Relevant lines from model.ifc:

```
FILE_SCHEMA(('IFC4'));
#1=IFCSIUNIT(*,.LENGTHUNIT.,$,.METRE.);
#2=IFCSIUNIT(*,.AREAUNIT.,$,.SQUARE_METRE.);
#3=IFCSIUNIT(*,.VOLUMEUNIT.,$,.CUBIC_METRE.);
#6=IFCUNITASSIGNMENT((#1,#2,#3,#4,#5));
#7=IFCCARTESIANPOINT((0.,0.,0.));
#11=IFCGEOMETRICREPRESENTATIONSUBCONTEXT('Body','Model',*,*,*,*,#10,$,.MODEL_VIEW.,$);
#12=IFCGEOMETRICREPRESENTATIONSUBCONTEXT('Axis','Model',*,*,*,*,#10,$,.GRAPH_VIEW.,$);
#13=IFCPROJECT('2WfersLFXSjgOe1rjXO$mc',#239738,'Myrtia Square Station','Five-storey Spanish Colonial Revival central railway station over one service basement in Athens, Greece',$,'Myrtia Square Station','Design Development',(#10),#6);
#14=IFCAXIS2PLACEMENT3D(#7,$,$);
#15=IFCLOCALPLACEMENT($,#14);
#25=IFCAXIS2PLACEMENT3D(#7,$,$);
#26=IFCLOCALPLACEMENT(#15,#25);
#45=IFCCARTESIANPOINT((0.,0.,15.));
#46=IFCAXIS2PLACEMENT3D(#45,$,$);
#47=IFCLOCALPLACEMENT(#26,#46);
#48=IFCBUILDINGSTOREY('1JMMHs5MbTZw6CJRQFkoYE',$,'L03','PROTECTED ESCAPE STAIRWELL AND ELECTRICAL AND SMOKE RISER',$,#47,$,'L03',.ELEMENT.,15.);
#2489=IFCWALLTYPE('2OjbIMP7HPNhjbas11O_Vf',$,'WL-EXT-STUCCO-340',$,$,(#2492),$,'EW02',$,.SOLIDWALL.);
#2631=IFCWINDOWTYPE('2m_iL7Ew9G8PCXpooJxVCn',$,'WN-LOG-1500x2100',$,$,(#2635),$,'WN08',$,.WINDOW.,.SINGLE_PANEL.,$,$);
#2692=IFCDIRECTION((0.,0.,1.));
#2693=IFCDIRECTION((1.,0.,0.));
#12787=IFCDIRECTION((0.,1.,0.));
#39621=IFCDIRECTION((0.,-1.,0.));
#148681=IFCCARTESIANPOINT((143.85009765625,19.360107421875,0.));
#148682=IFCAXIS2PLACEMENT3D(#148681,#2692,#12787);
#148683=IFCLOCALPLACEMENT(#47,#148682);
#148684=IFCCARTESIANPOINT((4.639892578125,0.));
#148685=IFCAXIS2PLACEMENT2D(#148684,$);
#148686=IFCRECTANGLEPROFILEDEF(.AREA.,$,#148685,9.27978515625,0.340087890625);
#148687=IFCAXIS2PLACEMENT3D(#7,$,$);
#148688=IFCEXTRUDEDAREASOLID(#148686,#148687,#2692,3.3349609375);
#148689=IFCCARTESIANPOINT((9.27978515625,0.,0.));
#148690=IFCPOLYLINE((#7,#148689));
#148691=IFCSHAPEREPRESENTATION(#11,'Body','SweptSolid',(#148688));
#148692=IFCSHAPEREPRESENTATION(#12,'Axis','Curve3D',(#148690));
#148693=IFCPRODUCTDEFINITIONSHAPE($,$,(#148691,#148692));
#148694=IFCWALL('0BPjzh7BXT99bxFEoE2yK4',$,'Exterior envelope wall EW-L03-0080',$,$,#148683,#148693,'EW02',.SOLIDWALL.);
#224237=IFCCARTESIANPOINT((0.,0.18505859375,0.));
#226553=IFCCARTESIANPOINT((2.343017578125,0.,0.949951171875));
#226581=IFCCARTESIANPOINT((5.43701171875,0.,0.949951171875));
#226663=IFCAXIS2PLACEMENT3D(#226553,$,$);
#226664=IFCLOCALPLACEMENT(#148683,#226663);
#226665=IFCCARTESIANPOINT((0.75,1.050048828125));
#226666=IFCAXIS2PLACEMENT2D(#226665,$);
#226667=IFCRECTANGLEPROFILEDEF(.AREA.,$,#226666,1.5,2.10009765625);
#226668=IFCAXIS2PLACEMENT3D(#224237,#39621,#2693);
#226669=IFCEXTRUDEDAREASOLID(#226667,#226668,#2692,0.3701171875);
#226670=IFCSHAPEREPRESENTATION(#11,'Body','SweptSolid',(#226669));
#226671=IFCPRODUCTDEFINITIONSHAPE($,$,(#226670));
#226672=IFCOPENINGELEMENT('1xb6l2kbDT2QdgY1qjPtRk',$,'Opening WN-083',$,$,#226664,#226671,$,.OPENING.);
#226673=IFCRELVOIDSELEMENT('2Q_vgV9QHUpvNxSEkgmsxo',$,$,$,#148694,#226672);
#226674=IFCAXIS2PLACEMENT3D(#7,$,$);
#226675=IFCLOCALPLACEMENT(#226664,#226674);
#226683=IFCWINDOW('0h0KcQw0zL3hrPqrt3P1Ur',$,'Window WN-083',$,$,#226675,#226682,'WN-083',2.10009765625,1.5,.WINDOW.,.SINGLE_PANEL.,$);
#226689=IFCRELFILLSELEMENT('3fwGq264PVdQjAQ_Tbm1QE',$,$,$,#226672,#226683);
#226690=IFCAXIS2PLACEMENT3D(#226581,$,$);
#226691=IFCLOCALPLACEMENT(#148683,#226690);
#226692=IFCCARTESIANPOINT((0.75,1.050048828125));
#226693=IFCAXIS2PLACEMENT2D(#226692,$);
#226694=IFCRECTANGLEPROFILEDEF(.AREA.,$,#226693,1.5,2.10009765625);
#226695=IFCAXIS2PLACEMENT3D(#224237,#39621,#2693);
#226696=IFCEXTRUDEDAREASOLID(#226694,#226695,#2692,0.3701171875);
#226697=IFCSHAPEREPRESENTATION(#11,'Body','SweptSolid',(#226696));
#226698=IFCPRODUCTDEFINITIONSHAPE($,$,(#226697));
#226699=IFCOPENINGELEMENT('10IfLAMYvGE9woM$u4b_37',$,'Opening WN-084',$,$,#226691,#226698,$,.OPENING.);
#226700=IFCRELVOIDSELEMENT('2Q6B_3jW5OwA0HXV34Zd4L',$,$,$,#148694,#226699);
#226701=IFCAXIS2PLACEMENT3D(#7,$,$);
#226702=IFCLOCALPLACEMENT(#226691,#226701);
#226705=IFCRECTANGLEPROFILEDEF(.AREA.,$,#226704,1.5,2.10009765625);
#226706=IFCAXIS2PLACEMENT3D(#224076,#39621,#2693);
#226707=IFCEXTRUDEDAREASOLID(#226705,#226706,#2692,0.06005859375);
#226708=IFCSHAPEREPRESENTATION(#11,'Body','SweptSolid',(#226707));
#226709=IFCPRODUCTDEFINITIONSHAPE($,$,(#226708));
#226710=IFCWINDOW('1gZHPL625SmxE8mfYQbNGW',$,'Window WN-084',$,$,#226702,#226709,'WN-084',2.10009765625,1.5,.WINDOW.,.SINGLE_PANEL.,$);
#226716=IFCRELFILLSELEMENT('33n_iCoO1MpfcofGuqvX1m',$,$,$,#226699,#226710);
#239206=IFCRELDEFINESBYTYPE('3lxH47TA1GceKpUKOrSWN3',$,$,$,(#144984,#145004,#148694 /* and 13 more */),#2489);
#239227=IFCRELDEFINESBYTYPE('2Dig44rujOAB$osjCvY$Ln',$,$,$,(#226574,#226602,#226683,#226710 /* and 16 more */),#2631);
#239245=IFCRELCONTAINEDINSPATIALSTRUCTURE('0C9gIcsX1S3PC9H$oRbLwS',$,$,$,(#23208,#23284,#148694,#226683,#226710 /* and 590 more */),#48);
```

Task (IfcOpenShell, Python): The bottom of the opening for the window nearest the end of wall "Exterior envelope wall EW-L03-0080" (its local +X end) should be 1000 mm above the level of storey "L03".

```python
import numpy as np
import ifcopenshell
import ifcopenshell.api.geometry
import ifcopenshell.geom
import ifcopenshell.util.element
import ifcopenshell.util.placement
import ifcopenshell.util.shape
import ifcopenshell.util.unit

model = ifcopenshell.open("model.ifc")
unit_scale = ifcopenshell.util.unit.calculate_unit_scale(model)

window = model.by_guid("1gZHPL625SmxE8mfYQbNGW")
opening = window.FillsVoids[0].RelatingOpeningElement
storey = ifcopenshell.util.element.get_container(window, ifc_class="IfcBuildingStorey")
level = ifcopenshell.util.placement.get_local_placement(storey.ObjectPlacement)[2, 3]

# The opening's origin need not be at the sill, so measure its lowest point.
shape = ifcopenshell.geom.create_shape(ifcopenshell.geom.settings(), opening)
bottom = ifcopenshell.util.shape.get_shape_bottom_elevation(shape, shape.geometry) / unit_scale
dz = level + 1 / unit_scale - bottom

shift = np.array([0.0, 0.0, dz])
# The window is placed relative to its opening, so it follows when the opening moves.
matrix = ifcopenshell.util.placement.get_local_placement(opening.ObjectPlacement)
matrix[:3, 3] += shift
ifcopenshell.api.geometry.edit_object_placement(
    model, product=opening, matrix=matrix, is_si=False, should_transform_children=True
)

print(f"moved by {dz * unit_scale:+.3f} m")

model.write("model-out.ifc")
```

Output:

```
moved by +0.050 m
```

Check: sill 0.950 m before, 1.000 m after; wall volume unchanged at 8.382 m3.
